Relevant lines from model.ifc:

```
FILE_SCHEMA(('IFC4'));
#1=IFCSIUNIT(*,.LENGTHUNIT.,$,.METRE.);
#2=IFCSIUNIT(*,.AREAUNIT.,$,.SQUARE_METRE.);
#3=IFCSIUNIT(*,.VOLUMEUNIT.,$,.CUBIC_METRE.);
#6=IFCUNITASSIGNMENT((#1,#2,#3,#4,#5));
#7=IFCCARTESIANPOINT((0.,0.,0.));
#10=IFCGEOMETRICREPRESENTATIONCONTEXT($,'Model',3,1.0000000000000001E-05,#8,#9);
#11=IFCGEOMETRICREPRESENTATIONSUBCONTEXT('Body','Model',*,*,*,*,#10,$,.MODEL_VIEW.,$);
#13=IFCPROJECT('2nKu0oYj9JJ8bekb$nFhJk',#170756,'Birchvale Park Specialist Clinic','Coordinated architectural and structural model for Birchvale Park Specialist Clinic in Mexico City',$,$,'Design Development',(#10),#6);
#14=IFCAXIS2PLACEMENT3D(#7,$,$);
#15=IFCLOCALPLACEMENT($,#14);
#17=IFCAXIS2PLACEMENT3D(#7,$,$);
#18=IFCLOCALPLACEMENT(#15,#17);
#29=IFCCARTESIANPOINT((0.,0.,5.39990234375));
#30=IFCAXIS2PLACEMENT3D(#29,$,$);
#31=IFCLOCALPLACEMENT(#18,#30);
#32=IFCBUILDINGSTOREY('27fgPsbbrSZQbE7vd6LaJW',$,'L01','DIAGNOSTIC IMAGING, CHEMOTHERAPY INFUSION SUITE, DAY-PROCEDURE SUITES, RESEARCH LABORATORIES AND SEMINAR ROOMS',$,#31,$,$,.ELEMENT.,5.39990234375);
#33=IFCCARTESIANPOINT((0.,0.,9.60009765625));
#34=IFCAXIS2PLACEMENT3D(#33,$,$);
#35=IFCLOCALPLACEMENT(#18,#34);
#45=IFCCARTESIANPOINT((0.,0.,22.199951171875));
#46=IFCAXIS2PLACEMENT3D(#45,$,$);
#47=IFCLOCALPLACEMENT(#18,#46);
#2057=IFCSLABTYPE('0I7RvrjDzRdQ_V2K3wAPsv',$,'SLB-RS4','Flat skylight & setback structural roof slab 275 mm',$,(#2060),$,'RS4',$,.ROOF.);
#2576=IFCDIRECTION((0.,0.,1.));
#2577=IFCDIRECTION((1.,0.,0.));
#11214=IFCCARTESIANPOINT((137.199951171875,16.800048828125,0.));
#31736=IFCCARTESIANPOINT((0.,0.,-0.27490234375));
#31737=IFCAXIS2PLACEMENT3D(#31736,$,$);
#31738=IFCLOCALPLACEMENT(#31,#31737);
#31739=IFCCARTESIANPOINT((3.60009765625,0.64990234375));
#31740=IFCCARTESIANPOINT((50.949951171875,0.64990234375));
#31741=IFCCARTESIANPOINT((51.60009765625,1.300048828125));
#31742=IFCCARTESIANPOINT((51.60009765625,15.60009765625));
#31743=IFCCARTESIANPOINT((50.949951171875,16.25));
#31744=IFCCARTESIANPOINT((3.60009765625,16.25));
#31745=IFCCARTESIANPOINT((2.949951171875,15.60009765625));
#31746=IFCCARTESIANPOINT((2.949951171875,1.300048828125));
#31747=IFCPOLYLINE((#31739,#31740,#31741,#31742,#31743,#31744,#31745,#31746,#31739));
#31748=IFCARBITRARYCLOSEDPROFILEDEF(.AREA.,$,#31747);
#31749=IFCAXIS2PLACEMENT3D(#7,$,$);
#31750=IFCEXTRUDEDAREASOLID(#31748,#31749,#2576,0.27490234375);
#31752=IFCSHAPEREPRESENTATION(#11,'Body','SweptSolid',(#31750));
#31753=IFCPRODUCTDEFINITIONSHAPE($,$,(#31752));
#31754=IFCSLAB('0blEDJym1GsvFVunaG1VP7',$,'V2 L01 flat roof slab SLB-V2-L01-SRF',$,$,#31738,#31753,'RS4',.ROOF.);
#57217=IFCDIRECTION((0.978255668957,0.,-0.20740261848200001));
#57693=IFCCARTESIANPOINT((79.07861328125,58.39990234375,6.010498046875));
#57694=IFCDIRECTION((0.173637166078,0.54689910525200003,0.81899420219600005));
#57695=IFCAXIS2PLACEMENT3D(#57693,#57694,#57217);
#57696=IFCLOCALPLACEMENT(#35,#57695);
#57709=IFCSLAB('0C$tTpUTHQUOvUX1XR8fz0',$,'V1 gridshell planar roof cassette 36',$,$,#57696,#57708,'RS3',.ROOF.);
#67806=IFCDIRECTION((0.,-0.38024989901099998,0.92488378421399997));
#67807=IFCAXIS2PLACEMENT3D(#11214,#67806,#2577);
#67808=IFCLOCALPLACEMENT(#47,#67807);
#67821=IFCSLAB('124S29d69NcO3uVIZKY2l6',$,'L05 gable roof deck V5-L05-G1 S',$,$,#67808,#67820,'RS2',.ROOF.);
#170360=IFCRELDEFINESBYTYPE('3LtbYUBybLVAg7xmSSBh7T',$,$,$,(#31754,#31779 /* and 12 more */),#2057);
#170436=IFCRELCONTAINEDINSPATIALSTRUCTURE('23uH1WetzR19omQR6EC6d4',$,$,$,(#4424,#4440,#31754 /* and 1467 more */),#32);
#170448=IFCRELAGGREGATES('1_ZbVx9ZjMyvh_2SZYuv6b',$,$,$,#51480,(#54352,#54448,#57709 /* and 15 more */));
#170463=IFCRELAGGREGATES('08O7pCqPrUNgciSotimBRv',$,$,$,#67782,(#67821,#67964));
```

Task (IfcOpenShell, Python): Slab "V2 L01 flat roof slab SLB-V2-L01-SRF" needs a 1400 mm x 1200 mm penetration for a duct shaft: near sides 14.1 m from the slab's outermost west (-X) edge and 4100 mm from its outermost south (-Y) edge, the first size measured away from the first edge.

```python
import numpy as np
import ifcopenshell
import ifcopenshell.api.feature
import ifcopenshell.api.geometry
import ifcopenshell.api.root
import ifcopenshell.geom
import ifcopenshell.util.placement
import ifcopenshell.util.representation
import ifcopenshell.util.shape
import ifcopenshell.util.unit

model = ifcopenshell.open("model.ifc")
unit_scale = ifcopenshell.util.unit.calculate_unit_scale(model)
settings = ifcopenshell.geom.settings()


def volume(element):
    """Net volume in cubic metres, openings subtracted."""
    shape = ifcopenshell.geom.create_shape(settings, element)
    return ifcopenshell.util.shape.get_volume(shape.geometry)


slab = model.by_guid("0blEDJym1GsvFVunaG1VP7")
before = volume(slab)

# Extent in the slab's own axes, in metres. The edges named are its -X and -Y sides.
slab_shape = ifcopenshell.geom.create_shape(settings, slab)
vertices = ifcopenshell.util.shape.get_vertices(slab_shape.geometry)
x_min, y_min, bottom = vertices.min(axis=0)
top = vertices[:, 2].max()

opening = ifcopenshell.api.root.create_entity(model, ifc_class="IfcOpeningElement", name="Duct shaft opening", predefined_type="OPENING")
context = ifcopenshell.util.representation.get_context(model, "Model", "Body", "MODEL_VIEW")
width, depth = 1.4, 1.2
outline = [(0.0, 0.0), (width, 0.0), (width, depth), (0.0, depth), (0.0, 0.0)]
# Overshoot both faces by 50 mm so the cut is clean.
shape = ifcopenshell.api.geometry.add_slab_representation(
    model, context=context, depth=top - bottom + 0.1, polyline=outline
)
ifcopenshell.api.geometry.assign_representation(model, product=opening, representation=shape)

matrix = ifcopenshell.util.placement.get_local_placement(slab.ObjectPlacement)
matrix[:, 3] = matrix @ np.append(np.array([x_min + 14.1, y_min + 4.1, bottom - 0.05]) / unit_scale, 1.0)
ifcopenshell.api.geometry.edit_object_placement(model, product=opening, matrix=matrix, is_si=False)
ifcopenshell.api.feature.add_feature(model, feature=opening, element=slab)

after = volume(slab)

print(f"slab volume {before:.3f} -> {after:.3f} m3")

model.write("model-out.ifc")
```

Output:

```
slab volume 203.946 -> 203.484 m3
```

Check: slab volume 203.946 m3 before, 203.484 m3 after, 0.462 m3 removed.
